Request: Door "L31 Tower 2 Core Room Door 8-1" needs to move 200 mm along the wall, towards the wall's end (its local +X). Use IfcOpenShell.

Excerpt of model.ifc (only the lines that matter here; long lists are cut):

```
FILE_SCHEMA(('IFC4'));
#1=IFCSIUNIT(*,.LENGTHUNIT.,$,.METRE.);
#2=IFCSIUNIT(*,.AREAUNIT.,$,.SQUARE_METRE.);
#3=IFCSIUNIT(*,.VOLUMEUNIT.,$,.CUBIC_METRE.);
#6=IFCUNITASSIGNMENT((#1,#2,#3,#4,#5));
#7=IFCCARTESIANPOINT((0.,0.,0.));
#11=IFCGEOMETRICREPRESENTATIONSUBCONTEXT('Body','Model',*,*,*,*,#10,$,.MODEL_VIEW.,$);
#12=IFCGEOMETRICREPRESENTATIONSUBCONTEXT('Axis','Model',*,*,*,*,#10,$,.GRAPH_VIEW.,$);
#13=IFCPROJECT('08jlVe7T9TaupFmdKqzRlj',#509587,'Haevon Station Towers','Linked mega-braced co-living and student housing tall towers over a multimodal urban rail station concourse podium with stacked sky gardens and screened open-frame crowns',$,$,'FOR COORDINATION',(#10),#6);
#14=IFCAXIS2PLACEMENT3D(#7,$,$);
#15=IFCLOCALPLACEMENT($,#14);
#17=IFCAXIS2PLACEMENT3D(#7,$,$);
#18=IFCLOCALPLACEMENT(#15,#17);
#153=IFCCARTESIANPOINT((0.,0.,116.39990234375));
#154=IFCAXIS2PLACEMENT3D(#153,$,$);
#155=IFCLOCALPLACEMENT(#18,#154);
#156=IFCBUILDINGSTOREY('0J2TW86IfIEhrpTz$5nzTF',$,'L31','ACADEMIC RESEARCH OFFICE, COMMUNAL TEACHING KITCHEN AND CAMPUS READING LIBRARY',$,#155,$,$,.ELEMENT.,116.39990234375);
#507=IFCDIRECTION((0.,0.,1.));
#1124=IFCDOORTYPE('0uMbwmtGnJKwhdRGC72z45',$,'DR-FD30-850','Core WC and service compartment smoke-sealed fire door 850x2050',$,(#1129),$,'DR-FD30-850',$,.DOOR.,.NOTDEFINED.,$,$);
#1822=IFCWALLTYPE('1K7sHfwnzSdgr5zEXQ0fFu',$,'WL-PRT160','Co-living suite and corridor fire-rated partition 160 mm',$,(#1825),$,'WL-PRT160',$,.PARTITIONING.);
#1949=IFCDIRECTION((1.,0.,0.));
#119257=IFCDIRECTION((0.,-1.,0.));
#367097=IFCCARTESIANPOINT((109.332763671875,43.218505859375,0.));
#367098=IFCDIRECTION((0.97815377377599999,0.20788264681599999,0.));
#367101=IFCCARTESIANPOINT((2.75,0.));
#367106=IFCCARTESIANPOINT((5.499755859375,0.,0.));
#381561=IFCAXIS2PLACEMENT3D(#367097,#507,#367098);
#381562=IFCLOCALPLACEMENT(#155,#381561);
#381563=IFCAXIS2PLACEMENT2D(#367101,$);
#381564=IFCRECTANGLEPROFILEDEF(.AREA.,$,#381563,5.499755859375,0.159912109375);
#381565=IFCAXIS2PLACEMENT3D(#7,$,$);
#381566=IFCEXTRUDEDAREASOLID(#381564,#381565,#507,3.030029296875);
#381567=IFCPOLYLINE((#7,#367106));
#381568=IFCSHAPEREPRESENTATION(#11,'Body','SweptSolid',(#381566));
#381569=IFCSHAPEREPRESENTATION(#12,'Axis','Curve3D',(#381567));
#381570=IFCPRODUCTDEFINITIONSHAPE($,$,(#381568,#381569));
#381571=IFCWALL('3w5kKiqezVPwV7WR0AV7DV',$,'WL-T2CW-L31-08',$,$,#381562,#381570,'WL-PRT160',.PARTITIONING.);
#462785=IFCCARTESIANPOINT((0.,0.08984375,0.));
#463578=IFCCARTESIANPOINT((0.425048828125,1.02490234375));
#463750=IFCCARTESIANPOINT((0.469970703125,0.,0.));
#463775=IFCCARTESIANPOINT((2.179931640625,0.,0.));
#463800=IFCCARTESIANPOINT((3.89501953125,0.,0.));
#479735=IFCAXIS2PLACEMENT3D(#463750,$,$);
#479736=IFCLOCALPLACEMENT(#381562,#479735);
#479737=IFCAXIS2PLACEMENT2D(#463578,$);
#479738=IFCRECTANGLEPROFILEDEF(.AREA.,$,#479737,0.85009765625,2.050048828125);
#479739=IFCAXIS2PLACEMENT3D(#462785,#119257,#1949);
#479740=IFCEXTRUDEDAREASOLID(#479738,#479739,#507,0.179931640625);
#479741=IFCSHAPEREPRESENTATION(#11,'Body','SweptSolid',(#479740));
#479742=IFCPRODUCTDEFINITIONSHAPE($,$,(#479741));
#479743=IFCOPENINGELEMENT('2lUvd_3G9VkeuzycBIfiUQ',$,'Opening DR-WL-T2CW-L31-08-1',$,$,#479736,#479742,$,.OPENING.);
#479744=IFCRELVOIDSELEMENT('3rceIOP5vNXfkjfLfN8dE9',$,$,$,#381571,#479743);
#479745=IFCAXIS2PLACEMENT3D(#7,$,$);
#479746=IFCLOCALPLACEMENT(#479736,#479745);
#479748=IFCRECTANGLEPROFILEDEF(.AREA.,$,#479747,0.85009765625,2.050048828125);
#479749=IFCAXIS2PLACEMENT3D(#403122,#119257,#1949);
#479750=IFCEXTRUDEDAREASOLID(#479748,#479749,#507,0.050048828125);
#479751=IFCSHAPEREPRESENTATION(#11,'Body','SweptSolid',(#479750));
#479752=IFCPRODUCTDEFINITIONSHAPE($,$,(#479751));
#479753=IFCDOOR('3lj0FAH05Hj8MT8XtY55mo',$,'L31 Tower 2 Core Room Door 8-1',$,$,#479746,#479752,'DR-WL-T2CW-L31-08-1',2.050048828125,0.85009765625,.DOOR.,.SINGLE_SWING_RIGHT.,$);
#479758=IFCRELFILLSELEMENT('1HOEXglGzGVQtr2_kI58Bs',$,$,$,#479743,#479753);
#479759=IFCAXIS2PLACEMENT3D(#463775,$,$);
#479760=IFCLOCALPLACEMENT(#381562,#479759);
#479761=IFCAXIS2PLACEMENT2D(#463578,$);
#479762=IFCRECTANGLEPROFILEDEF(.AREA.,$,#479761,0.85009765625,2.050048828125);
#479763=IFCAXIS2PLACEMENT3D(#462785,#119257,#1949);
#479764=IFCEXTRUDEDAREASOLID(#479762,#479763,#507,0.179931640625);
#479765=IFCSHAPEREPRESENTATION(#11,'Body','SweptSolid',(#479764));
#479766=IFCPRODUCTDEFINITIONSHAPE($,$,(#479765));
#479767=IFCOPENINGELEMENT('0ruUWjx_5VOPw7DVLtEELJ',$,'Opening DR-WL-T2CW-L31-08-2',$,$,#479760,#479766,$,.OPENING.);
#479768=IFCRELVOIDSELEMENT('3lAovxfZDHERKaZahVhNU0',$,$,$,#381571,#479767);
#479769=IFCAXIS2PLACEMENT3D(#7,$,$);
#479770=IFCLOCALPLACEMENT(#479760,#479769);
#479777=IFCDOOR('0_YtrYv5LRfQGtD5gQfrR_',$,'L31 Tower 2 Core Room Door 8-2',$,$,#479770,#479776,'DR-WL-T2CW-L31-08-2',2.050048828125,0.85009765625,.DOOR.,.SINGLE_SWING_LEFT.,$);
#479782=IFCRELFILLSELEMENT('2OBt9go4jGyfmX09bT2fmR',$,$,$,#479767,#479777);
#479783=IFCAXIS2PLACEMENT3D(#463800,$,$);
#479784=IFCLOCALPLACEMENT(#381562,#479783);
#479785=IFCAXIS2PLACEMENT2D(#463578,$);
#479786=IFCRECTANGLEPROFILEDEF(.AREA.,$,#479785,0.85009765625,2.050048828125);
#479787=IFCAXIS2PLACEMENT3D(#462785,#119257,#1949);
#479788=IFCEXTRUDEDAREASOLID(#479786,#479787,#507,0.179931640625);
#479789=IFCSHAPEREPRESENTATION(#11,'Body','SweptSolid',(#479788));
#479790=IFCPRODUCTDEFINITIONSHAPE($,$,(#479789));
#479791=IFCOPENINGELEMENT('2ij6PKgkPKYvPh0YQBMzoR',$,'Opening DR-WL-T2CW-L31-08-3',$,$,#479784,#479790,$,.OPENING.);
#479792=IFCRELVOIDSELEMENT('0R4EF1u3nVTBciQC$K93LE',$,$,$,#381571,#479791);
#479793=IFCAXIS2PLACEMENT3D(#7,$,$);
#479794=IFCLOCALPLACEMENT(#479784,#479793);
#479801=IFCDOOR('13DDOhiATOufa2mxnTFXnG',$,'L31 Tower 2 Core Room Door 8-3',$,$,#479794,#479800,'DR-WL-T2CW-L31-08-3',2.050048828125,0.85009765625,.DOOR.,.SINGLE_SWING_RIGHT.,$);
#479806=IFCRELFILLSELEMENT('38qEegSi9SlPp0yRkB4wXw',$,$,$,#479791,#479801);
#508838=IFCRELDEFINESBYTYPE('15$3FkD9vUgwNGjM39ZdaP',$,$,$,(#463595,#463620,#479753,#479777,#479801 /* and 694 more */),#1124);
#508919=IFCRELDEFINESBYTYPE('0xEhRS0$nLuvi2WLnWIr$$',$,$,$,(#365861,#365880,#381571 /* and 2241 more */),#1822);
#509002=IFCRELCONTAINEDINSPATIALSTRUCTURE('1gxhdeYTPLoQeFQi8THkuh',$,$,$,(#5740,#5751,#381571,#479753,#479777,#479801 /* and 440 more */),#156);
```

```python
import ifcopenshell
import ifcopenshell.api.geometry
import ifcopenshell.util.placement
import ifcopenshell.util.unit

model = ifcopenshell.open("model.ifc")
unit_scale = ifcopenshell.util.unit.calculate_unit_scale(model)

door = model.by_guid("3lj0FAH05Hj8MT8XtY55mo")
opening = door.FillsVoids[0].RelatingOpeningElement
wall = opening.VoidsElements[0].RelatingBuildingElement

wall_matrix = ifcopenshell.util.placement.get_local_placement(wall.ObjectPlacement)
shift = wall_matrix[:3, 0] * 0.2 / unit_scale
before = ifcopenshell.util.placement.get_local_placement(door.ObjectPlacement)[:3, 3].copy()

# The door is placed relative to its opening, so it follows when the opening moves.
matrix = ifcopenshell.util.placement.get_local_placement(opening.ObjectPlacement)
matrix[:3, 3] += shift
ifcopenshell.api.geometry.edit_object_placement(
    model, product=opening, matrix=matrix, is_si=False, should_transform_children=True
)

after = ifcopenshell.util.placement.get_local_placement(door.ObjectPlacement)[:3, 3]
print("door moved by", (after - before).round(3) + 0.0)

model.write("model_v2.ifc")
```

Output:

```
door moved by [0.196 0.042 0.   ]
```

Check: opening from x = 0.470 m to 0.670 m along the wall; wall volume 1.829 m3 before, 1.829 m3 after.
